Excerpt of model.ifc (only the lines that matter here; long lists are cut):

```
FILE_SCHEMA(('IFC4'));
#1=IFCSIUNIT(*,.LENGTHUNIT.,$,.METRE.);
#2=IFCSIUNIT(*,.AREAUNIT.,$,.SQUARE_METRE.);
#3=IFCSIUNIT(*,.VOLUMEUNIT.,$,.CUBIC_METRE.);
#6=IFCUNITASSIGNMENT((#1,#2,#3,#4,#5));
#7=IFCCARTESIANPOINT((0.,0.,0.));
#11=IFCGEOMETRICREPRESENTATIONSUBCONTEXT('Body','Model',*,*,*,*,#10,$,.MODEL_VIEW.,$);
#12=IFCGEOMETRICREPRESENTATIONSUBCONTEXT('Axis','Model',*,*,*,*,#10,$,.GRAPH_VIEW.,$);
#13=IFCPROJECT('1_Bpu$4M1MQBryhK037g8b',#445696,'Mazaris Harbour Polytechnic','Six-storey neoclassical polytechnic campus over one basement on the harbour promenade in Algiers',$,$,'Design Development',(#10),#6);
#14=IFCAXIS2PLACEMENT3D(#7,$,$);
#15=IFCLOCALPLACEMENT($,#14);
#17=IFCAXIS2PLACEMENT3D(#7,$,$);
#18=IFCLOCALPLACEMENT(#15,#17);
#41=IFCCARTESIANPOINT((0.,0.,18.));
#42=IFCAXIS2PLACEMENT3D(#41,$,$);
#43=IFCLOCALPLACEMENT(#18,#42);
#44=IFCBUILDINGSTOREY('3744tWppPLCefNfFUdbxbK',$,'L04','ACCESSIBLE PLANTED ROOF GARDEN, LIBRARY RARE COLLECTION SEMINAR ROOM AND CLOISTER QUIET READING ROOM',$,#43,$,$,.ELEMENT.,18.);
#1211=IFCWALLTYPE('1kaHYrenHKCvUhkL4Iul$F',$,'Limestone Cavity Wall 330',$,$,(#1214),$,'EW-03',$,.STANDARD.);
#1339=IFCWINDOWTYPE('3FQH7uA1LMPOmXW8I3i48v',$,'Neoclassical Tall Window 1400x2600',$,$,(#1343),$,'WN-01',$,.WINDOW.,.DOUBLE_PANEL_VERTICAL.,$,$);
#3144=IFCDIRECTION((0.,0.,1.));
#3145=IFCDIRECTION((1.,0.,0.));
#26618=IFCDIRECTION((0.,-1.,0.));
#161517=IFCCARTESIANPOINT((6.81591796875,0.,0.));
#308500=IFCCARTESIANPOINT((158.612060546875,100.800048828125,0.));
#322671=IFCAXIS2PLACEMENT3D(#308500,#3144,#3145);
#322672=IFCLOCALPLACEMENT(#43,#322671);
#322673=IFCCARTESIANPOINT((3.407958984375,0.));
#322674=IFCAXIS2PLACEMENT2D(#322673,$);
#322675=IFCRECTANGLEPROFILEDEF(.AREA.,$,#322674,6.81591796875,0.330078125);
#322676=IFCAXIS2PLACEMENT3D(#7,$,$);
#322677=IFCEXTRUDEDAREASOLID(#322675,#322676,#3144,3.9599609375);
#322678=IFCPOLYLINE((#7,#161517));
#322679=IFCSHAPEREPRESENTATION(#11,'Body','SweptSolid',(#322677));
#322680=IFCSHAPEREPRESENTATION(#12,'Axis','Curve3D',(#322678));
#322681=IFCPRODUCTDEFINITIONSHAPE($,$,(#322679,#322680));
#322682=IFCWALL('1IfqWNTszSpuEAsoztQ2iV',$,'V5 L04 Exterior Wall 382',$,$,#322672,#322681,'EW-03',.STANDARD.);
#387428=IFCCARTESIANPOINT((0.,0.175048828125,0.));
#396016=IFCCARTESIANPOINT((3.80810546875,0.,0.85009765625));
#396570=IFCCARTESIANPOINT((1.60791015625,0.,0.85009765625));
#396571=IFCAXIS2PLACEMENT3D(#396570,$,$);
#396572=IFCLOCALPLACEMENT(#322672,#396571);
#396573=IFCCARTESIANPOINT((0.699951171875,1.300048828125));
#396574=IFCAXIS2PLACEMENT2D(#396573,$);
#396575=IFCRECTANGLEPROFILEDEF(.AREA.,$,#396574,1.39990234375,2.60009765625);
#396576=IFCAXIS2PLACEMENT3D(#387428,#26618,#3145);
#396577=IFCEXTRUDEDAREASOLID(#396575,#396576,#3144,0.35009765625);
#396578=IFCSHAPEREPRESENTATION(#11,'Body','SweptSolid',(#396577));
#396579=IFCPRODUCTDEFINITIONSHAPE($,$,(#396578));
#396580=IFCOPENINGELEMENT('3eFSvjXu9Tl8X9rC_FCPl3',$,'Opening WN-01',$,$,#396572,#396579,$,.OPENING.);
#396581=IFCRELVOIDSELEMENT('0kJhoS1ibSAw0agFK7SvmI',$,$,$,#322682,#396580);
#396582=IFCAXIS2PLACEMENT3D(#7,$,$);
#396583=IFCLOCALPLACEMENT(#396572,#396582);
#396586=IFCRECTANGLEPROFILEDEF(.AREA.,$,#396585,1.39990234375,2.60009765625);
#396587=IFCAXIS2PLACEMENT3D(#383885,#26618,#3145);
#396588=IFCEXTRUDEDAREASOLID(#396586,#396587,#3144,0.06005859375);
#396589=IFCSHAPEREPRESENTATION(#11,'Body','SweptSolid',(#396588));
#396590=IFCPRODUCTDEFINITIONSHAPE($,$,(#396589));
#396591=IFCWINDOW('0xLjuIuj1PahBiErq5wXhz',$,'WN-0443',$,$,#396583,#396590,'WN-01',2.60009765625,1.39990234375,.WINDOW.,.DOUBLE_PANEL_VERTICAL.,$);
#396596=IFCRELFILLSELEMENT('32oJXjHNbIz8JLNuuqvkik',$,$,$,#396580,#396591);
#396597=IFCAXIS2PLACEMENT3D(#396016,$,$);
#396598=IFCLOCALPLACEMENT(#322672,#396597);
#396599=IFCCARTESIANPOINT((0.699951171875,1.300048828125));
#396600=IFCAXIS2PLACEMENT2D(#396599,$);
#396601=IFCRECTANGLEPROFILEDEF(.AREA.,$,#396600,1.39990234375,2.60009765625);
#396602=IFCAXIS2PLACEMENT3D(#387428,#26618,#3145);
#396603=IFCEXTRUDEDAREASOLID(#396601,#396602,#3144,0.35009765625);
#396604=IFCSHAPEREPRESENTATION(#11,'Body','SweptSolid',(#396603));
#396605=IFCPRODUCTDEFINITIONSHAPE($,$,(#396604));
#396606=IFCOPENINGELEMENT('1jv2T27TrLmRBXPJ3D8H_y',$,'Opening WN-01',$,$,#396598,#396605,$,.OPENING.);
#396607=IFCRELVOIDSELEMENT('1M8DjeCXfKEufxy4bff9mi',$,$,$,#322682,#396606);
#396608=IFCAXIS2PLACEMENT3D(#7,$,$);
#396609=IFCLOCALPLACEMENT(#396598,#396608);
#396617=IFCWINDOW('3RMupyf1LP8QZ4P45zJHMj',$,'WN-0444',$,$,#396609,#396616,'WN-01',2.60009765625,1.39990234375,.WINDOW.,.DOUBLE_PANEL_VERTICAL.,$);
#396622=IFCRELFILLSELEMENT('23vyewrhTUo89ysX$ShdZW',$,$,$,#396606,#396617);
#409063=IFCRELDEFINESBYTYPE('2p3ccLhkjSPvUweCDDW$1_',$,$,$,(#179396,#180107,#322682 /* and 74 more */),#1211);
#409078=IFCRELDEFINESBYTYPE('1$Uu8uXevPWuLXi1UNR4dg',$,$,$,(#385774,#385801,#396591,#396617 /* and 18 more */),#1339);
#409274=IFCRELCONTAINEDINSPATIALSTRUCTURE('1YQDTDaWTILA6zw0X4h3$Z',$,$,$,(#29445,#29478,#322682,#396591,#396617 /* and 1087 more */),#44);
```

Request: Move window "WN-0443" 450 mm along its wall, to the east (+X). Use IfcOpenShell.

```python
import ifcopenshell
import ifcopenshell.api.geometry
import ifcopenshell.util.placement
import ifcopenshell.util.unit

model = ifcopenshell.open("model.ifc")
unit_scale = ifcopenshell.util.unit.calculate_unit_scale(model)

window = model.by_guid("0xLjuIuj1PahBiErq5wXhz")
opening = window.FillsVoids[0].RelatingOpeningElement
wall = opening.VoidsElements[0].RelatingBuildingElement

wall_matrix = ifcopenshell.util.placement.get_local_placement(wall.ObjectPlacement)
shift = wall_matrix[:3, 0] * 0.45 / unit_scale
before = ifcopenshell.util.placement.get_local_placement(window.ObjectPlacement)[:3, 3].copy()

# The window is placed relative to its opening, so it follows when the opening moves.
matrix = ifcopenshell.util.placement.get_local_placement(opening.ObjectPlacement)
matrix[:3, 3] += shift
ifcopenshell.api.geometry.edit_object_placement(
    model, product=opening, matrix=matrix, is_si=False, should_transform_children=True
)

after = ifcopenshell.util.placement.get_local_placement(window.ObjectPlacement)[:3, 3]
print("window moved by", (after - before).round(3) + 0.0)

model.write("model-out.ifc")
```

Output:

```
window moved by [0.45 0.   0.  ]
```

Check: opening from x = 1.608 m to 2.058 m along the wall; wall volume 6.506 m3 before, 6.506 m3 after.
